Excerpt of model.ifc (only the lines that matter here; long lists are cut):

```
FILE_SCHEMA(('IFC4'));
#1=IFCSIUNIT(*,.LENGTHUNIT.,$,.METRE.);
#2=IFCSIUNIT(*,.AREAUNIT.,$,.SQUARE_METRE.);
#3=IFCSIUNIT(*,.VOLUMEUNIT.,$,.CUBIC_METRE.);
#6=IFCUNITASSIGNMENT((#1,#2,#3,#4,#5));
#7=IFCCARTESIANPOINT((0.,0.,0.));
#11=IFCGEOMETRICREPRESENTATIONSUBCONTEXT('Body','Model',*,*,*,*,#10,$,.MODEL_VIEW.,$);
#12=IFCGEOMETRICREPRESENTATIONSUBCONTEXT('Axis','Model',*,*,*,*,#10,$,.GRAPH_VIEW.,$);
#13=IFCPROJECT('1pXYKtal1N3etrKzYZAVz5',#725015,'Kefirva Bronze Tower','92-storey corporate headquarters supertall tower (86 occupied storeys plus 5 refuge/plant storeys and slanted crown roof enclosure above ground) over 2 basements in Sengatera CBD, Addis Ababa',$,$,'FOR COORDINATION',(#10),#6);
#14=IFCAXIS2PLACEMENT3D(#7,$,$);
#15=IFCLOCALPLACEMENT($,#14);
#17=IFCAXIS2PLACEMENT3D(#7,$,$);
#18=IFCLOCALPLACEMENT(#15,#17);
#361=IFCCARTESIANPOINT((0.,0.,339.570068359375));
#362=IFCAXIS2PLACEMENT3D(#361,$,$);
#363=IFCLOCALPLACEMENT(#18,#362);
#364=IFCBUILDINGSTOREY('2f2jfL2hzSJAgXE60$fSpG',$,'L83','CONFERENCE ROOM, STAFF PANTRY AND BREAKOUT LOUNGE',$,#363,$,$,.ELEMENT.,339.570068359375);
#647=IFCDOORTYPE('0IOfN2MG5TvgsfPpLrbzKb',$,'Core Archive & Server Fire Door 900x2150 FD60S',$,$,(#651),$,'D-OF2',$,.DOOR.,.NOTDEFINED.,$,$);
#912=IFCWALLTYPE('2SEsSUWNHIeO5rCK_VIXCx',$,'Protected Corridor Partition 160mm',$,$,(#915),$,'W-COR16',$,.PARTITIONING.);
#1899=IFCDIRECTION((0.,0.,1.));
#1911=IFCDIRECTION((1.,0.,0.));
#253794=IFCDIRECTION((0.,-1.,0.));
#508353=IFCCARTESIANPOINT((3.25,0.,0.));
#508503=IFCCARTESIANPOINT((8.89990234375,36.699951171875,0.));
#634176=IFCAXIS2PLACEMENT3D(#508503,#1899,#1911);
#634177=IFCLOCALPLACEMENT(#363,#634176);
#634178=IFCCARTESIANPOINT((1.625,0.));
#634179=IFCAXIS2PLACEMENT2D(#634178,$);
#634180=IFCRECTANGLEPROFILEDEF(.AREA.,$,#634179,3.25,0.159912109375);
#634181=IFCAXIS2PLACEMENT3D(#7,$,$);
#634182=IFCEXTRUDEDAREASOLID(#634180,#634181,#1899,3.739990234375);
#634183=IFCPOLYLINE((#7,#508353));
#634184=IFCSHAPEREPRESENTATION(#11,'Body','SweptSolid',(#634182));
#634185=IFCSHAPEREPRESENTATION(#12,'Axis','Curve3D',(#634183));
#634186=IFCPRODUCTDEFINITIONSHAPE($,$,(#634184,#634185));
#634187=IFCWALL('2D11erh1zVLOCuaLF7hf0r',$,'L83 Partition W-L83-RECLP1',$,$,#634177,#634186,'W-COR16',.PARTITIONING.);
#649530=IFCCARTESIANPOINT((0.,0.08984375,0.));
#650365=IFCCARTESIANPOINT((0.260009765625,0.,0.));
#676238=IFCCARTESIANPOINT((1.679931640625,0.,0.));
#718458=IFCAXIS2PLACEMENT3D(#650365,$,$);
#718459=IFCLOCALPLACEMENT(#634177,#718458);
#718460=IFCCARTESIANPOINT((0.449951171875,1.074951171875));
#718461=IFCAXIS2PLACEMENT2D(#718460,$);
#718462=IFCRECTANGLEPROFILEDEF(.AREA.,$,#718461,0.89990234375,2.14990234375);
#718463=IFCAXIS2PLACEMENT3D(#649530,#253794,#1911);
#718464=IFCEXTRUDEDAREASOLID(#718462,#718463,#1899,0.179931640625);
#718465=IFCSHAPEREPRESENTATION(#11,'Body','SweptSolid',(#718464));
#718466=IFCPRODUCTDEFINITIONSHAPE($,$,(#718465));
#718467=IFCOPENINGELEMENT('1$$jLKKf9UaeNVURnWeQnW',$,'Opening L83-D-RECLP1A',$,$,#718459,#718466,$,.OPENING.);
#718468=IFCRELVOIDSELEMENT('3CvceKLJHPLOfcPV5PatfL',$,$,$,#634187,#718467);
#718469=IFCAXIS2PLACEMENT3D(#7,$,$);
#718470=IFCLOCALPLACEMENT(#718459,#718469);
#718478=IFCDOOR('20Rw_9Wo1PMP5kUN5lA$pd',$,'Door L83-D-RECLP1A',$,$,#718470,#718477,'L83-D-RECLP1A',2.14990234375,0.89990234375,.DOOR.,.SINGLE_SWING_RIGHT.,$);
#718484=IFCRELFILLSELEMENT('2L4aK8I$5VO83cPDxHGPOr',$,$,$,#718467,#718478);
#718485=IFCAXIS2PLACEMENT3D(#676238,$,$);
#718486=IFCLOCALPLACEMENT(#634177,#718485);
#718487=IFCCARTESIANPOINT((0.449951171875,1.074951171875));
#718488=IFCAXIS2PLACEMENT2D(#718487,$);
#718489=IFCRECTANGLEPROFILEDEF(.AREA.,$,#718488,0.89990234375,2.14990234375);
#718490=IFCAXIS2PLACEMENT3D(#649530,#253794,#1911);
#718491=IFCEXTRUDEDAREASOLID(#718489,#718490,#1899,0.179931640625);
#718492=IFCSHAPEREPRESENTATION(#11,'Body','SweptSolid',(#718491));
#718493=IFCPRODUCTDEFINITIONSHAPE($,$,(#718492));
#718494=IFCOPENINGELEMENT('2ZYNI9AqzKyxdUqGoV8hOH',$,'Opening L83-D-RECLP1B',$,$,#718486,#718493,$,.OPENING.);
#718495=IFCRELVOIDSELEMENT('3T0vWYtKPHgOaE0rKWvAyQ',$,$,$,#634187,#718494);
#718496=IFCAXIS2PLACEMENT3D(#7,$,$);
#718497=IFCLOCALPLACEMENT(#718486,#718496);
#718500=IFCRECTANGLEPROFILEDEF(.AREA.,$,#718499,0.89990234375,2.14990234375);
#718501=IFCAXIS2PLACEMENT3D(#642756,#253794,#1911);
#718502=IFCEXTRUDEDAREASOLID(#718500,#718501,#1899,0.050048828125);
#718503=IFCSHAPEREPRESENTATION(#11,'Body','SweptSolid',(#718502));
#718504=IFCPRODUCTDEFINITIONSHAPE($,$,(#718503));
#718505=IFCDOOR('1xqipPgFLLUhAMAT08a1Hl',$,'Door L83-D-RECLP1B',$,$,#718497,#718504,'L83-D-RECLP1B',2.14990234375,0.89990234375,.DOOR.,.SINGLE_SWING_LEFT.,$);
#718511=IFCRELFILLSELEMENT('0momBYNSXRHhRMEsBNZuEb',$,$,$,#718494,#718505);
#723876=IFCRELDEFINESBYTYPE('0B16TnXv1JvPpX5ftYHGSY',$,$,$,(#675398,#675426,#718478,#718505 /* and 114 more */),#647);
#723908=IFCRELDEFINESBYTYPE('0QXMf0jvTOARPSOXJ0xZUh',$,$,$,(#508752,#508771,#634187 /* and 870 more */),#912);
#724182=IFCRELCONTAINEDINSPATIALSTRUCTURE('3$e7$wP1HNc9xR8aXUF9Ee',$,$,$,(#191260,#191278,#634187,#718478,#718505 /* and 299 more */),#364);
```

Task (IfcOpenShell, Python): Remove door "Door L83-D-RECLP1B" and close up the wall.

```python
import ifcopenshell
import ifcopenshell.api.feature
import ifcopenshell.api.root
import ifcopenshell.geom
import ifcopenshell.util.shape

model = ifcopenshell.open("model.ifc")
settings = ifcopenshell.geom.settings()


def volume(element):
    """Net volume in cubic metres, openings subtracted."""
    shape = ifcopenshell.geom.create_shape(settings, element)
    return ifcopenshell.util.shape.get_volume(shape.geometry)


door = model.by_guid("1xqipPgFLLUhAMAT08a1Hl")
opening = door.FillsVoids[0].RelatingOpeningElement
wall = opening.VoidsElements[0].RelatingBuildingElement
before = volume(wall)

ifcopenshell.api.root.remove_product(model, product=door)
ifcopenshell.api.feature.remove_feature(model, feature=opening)

after = volume(wall)

print(f"wall volume {before:.3f} -> {after:.3f} m3")

model.write("model_edited.ifc")
```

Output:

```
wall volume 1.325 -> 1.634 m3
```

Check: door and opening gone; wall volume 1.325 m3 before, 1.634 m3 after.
